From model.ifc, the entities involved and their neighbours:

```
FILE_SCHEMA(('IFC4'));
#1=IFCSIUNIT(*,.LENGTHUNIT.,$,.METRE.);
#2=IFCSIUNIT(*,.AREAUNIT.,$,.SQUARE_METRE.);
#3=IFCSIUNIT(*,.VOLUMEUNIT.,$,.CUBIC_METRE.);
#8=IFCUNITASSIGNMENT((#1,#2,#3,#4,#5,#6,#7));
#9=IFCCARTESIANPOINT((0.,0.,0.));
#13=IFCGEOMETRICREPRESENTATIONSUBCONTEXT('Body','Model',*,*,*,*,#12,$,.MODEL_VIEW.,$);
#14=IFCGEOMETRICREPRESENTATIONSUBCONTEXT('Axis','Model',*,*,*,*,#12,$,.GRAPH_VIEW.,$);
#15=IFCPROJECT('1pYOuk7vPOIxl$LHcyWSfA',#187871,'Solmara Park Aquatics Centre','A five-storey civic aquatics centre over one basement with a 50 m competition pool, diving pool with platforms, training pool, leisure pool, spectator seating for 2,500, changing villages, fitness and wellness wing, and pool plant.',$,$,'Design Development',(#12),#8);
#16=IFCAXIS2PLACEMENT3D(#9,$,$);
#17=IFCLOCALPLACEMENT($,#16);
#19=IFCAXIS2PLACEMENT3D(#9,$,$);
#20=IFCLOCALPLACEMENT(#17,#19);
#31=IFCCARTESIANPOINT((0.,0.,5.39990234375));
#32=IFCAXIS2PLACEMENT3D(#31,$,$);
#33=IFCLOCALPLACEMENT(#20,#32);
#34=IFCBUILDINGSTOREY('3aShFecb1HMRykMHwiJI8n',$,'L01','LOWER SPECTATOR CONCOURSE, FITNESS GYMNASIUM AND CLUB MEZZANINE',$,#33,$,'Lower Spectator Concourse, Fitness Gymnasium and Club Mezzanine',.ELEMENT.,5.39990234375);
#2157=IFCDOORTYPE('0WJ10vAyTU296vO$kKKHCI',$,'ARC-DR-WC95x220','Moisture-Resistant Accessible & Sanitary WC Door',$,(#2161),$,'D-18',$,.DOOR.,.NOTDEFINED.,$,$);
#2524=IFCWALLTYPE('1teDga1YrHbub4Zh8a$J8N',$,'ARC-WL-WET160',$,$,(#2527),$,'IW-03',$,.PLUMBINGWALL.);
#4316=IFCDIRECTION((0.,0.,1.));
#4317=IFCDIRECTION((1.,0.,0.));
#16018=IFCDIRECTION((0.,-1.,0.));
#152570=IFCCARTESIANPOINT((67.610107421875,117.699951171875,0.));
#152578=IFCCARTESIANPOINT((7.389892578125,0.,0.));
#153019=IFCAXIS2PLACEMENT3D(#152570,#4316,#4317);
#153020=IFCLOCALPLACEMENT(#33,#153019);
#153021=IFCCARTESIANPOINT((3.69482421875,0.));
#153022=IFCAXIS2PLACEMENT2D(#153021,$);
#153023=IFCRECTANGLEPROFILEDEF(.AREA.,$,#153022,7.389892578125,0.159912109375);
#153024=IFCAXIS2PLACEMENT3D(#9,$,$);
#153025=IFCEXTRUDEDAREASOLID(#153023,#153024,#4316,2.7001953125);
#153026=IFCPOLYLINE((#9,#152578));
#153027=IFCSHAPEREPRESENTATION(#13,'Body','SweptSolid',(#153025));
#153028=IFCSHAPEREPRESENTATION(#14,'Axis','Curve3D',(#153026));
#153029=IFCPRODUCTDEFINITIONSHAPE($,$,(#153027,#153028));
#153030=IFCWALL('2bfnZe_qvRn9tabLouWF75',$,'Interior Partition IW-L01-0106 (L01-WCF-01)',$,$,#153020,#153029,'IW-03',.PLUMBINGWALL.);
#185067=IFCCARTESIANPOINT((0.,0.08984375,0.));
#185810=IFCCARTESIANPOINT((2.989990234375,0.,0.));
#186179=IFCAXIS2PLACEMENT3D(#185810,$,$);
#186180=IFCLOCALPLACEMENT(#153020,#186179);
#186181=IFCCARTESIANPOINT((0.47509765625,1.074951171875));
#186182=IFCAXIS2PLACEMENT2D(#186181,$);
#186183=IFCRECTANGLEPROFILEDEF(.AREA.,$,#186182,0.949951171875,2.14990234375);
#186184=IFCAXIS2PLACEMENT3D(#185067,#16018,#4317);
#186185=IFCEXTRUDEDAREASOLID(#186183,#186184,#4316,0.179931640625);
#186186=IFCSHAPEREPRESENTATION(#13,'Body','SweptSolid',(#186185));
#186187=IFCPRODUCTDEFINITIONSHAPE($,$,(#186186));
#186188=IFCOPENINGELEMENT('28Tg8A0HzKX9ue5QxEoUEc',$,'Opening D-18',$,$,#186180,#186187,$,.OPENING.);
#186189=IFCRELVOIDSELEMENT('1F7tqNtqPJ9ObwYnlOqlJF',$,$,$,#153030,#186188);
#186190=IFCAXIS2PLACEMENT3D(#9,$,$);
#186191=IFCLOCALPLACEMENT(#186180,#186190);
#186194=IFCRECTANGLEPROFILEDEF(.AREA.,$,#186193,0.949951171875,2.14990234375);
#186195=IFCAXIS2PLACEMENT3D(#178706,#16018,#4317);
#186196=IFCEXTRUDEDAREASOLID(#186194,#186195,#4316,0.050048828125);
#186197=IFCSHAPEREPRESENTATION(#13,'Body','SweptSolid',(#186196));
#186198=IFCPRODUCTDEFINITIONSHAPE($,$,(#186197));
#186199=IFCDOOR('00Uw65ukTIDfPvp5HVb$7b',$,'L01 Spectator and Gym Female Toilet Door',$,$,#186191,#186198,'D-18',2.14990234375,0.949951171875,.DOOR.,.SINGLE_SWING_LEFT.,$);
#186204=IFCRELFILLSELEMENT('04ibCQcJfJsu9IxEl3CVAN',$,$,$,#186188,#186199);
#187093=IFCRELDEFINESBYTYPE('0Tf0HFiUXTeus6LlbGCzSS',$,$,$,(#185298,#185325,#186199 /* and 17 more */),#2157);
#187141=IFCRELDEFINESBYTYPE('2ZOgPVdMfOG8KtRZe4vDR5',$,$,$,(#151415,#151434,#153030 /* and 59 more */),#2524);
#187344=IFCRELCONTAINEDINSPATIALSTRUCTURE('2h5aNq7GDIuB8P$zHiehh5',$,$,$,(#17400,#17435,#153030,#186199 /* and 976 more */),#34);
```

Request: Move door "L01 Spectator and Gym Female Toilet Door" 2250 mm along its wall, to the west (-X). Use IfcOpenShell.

```python
import ifcopenshell
import ifcopenshell.api.geometry
import ifcopenshell.util.placement
import ifcopenshell.util.unit

model = ifcopenshell.open("model.ifc")
unit_scale = ifcopenshell.util.unit.calculate_unit_scale(model)

door = model.by_guid("00Uw65ukTIDfPvp5HVb$7b")
opening = door.FillsVoids[0].RelatingOpeningElement
wall = opening.VoidsElements[0].RelatingBuildingElement

wall_matrix = ifcopenshell.util.placement.get_local_placement(wall.ObjectPlacement)
shift = wall_matrix[:3, 0] * -2.25 / unit_scale
before = ifcopenshell.util.placement.get_local_placement(door.ObjectPlacement)[:3, 3].copy()

# The door is placed relative to its opening, so it follows when the opening moves.
matrix = ifcopenshell.util.placement.get_local_placement(opening.ObjectPlacement)
matrix[:3, 3] += shift
ifcopenshell.api.geometry.edit_object_placement(
    model, product=opening, matrix=matrix, is_si=False, should_transform_children=True
)

after = ifcopenshell.util.placement.get_local_placement(door.ObjectPlacement)[:3, 3]
print("door moved by", (after - before).round(3) + 0.0)

model.write("model-out.ifc")
```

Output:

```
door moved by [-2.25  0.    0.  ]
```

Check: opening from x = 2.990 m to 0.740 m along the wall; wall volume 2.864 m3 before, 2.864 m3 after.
